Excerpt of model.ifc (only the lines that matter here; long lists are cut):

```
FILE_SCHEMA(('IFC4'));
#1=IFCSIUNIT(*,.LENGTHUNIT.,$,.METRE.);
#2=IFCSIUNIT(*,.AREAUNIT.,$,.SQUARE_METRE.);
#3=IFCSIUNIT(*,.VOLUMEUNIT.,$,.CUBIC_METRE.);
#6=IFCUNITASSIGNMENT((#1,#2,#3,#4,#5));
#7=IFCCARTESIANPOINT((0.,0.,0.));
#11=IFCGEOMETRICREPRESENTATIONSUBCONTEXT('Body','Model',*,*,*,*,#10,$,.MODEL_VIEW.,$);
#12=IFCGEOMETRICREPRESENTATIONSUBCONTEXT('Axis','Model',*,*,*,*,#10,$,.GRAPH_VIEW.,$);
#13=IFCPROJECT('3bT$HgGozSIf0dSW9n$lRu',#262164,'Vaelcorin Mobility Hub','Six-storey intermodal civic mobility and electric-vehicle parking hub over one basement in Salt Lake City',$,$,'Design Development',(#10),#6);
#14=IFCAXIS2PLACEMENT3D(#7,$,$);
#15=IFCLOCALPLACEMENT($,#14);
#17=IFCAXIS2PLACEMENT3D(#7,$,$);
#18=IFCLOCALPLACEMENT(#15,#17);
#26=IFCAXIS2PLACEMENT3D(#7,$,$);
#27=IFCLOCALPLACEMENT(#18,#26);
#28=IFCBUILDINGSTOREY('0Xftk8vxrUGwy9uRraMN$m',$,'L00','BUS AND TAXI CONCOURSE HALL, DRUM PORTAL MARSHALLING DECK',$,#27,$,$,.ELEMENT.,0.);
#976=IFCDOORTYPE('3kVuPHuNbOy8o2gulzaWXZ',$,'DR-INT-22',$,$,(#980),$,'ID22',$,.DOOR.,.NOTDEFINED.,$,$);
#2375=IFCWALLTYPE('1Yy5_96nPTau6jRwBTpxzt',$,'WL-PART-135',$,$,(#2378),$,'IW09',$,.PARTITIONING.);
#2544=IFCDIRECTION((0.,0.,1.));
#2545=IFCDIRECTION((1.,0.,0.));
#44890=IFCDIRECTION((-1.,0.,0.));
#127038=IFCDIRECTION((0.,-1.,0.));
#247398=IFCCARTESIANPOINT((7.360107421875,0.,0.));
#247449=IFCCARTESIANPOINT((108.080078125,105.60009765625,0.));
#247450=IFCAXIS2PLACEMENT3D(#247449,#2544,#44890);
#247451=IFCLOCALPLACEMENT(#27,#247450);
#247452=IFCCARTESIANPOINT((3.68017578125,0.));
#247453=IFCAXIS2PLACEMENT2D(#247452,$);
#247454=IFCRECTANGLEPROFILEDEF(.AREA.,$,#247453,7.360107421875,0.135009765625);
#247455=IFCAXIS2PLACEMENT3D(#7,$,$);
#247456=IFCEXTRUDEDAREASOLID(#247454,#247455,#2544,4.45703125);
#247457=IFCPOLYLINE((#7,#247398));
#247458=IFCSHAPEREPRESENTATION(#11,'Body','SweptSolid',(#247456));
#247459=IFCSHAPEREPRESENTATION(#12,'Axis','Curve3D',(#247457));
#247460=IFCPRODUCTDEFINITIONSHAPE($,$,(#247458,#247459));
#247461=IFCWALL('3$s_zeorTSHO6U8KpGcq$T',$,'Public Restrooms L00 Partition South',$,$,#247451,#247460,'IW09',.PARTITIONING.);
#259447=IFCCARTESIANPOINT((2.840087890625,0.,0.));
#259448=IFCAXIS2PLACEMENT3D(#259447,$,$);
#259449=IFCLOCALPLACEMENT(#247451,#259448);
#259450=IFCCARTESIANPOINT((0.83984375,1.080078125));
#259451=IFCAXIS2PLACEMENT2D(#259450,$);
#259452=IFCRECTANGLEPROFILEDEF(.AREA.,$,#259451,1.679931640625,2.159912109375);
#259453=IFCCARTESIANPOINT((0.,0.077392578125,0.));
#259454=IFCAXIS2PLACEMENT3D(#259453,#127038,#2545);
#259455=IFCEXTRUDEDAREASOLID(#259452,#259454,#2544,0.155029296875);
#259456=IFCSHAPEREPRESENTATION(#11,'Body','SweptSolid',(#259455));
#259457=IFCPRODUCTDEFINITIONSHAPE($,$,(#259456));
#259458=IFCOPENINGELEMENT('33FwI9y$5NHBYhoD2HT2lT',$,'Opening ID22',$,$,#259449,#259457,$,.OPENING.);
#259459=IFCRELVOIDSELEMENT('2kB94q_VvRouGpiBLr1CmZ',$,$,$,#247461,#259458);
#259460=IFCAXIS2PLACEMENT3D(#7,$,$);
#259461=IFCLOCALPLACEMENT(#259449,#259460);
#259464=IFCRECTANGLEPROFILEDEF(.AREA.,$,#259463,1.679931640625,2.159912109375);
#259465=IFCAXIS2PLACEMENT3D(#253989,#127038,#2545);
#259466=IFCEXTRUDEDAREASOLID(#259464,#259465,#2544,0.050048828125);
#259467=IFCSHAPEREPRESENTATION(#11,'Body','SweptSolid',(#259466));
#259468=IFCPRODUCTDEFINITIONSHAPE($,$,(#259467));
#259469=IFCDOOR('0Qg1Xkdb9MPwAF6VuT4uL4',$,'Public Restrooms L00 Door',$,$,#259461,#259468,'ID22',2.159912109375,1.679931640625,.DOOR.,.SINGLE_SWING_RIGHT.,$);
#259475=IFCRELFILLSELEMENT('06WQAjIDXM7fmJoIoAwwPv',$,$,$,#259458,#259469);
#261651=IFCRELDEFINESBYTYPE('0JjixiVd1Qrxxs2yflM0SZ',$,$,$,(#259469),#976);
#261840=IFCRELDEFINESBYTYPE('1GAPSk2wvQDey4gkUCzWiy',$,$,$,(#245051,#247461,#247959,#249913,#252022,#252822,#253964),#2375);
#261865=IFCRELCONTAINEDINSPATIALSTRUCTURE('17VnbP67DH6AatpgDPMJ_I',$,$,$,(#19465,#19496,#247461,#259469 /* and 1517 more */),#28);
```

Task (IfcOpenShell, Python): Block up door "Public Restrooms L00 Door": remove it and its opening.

```python
import ifcopenshell
import ifcopenshell.api.feature
import ifcopenshell.api.root
import ifcopenshell.geom
import ifcopenshell.util.shape

model = ifcopenshell.open("model.ifc")
settings = ifcopenshell.geom.settings()


def volume(element):
    """Net volume in cubic metres, openings subtracted."""
    shape = ifcopenshell.geom.create_shape(settings, element)
    return ifcopenshell.util.shape.get_volume(shape.geometry)


door = model.by_guid("0Qg1Xkdb9MPwAF6VuT4uL4")
opening = door.FillsVoids[0].RelatingOpeningElement
wall = opening.VoidsElements[0].RelatingBuildingElement
before = volume(wall)

ifcopenshell.api.root.remove_product(model, product=door)
ifcopenshell.api.feature.remove_feature(model, feature=opening)

after = volume(wall)

print(f"wall volume {before:.3f} -> {after:.3f} m3")

model.write("model_rev.ifc")
```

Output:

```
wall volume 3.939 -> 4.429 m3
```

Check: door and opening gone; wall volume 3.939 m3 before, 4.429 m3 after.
